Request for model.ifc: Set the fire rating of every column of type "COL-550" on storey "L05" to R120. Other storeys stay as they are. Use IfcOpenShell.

First a look at what the model holds.

```python
import ifcopenshell
import ifcopenshell.util.element

model = ifcopenshell.open("model.ifc")
print(model.schema)
storey = next(s for s in model.by_type("IfcBuildingStorey") if s.Name == "L05")
columns = [e for e in ifcopenshell.util.element.get_decomposition(storey) if e.is_a("IfcColumn")]
seen = {}
for e in columns:
    element_type = ifcopenshell.util.element.get_type(e)
    key = (element_type.Name if element_type != e and element_type else None, ifcopenshell.util.element.get_pset(e, "Pset_ColumnCommon", "FireRating"))
    seen[key] = seen.get(key, 0) + 1
for (name, value), count in sorted(seen.items(), key=str):
    print(count, "x", name, "|", value)
```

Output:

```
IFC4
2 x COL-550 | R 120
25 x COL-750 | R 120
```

```python
import ifcopenshell
import ifcopenshell.api.pset
import ifcopenshell.util.element

model = ifcopenshell.open("model.ifc")

storey = next(s for s in model.by_type("IfcBuildingStorey") if s.Name == "L05")
columns = [e for e in ifcopenshell.util.element.get_decomposition(storey) if e.is_a("IfcColumn")]

count = 0
for e in columns:
    element_type = ifcopenshell.util.element.get_type(e)
    if element_type in (None, e) or element_type.Name != "COL-550":
        continue
    # add_pset returns the element's existing set when there is one.
    pset = ifcopenshell.api.pset.add_pset(model, product=e, name="Pset_ColumnCommon")
    ifcopenshell.api.pset.edit_pset(model, pset=pset, properties={"FireRating": "R120"})
    count += 1

print(count, "columns updated")

model.write("model_edited.ifc")
```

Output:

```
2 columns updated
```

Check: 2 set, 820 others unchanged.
